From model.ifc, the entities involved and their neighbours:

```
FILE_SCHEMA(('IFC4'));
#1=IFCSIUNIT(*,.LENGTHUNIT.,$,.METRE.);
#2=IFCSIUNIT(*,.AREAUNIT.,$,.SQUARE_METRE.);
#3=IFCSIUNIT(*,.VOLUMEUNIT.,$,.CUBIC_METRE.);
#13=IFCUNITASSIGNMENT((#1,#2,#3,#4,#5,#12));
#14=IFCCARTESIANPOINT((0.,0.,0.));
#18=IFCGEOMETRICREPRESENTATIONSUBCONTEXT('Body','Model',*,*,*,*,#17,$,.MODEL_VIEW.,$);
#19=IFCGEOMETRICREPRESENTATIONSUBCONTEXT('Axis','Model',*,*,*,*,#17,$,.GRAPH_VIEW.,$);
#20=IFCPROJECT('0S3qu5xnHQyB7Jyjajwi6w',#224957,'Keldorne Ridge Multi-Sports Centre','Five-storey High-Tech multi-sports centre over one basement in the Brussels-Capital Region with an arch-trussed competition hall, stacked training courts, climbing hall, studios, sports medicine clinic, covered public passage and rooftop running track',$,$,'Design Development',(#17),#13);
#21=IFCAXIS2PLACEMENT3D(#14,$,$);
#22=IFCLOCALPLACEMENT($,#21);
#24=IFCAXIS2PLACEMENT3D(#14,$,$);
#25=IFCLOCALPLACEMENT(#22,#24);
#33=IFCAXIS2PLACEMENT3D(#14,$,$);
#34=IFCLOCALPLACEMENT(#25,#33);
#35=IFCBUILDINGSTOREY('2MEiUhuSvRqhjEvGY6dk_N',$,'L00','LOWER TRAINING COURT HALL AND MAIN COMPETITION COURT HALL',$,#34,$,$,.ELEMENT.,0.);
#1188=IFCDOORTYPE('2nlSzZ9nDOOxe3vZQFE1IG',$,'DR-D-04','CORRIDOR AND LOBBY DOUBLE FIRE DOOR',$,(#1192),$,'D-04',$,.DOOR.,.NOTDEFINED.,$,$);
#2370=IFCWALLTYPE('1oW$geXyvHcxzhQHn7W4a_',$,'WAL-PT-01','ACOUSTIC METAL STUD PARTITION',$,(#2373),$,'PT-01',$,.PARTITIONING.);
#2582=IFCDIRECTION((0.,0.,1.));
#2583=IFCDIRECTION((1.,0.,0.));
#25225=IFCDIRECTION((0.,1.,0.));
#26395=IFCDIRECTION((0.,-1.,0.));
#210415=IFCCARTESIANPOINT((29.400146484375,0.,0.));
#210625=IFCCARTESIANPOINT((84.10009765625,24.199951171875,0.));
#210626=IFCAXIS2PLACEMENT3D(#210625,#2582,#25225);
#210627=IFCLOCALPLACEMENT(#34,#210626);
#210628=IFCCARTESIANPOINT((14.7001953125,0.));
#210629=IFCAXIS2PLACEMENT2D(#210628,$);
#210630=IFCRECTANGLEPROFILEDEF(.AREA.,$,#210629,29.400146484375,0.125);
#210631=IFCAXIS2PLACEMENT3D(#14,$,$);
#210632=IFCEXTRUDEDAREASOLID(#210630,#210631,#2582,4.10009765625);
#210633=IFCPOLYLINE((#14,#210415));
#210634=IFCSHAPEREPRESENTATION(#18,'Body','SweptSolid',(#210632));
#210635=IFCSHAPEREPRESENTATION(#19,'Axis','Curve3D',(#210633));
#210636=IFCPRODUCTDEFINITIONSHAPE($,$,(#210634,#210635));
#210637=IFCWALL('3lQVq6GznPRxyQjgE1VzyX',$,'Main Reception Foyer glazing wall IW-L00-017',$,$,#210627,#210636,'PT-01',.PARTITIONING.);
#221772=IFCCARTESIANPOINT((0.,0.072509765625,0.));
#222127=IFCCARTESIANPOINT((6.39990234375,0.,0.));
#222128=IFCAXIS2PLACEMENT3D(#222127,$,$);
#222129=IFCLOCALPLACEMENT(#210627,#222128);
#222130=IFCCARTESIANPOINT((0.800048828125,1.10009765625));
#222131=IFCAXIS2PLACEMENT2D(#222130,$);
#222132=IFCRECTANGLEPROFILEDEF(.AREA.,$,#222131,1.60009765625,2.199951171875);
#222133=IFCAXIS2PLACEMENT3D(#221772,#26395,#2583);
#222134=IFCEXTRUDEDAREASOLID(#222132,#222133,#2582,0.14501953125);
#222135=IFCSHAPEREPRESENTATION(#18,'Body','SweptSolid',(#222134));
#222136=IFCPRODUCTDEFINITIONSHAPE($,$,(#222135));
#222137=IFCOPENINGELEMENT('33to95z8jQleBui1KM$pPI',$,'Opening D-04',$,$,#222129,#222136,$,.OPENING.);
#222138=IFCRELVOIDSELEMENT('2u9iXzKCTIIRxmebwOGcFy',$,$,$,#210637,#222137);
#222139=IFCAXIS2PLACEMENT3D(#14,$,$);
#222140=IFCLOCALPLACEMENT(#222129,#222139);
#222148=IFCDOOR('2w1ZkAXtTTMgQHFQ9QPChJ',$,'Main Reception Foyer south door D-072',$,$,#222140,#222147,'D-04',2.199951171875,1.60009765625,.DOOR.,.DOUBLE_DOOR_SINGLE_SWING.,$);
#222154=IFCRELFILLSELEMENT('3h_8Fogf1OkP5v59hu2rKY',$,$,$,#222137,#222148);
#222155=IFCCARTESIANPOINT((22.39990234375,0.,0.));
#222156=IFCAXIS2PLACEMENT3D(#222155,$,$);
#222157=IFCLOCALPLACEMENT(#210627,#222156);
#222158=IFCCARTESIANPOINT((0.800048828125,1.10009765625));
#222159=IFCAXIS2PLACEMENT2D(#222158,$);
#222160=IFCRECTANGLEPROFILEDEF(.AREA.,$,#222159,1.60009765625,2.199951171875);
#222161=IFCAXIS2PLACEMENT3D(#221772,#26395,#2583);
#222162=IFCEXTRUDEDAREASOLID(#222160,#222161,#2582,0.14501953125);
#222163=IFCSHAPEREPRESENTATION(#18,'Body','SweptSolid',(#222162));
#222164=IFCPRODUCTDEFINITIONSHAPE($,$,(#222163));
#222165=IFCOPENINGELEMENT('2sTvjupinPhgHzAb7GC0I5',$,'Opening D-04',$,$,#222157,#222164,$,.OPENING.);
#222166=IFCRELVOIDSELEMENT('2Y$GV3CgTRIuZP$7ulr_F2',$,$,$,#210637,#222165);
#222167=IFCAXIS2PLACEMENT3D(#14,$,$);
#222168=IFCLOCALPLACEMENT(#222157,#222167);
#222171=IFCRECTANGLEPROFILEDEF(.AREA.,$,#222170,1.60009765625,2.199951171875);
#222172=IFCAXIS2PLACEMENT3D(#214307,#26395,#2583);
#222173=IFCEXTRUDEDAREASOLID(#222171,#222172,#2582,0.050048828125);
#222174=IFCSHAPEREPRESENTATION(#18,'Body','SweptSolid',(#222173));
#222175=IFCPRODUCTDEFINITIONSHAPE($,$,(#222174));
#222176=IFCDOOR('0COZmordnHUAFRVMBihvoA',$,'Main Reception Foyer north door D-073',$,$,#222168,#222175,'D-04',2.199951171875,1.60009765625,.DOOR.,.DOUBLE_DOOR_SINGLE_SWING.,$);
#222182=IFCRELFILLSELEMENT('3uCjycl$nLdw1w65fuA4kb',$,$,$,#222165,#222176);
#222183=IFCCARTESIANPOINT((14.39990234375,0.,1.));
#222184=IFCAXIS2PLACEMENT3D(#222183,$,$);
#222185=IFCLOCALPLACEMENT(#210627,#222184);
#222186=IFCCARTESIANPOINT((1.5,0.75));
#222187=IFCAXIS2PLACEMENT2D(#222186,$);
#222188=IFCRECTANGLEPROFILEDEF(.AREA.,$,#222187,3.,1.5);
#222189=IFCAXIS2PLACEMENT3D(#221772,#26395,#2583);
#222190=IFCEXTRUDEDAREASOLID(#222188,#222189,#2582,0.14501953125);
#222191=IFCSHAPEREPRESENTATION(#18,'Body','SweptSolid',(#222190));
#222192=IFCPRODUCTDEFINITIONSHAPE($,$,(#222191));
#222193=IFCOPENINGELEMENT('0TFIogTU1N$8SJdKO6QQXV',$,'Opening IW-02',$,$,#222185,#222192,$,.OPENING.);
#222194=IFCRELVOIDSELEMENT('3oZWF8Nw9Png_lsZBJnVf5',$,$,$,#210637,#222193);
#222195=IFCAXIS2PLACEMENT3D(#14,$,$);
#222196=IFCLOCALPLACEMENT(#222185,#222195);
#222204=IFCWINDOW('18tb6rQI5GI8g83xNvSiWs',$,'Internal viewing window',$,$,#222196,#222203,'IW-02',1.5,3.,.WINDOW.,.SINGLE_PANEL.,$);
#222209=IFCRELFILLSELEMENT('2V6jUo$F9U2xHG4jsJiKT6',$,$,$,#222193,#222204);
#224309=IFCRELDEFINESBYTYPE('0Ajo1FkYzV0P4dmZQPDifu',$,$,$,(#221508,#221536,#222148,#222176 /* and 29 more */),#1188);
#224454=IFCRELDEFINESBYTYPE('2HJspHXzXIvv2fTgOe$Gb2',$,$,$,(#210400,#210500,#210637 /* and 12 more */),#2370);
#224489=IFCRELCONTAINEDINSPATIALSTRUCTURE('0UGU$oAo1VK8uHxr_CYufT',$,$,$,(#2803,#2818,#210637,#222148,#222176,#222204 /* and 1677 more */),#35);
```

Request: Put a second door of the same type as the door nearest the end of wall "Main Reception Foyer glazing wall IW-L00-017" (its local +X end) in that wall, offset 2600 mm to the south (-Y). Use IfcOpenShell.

```python
import ifcopenshell
import ifcopenshell.api.feature
import ifcopenshell.api.geometry
import ifcopenshell.api.root
import ifcopenshell.geom
import ifcopenshell.util.element
import ifcopenshell.util.placement
import ifcopenshell.util.shape
import ifcopenshell.util.unit

model = ifcopenshell.open("model.ifc")
unit_scale = ifcopenshell.util.unit.calculate_unit_scale(model)
settings = ifcopenshell.geom.settings()


def volume(element):
    """Net volume in cubic metres, openings subtracted."""
    shape = ifcopenshell.geom.create_shape(settings, element)
    return ifcopenshell.util.shape.get_volume(shape.geometry)


door = model.by_guid("0COZmordnHUAFRVMBihvoA")
opening = door.FillsVoids[0].RelatingOpeningElement
wall = opening.VoidsElements[0].RelatingBuildingElement
before = volume(wall)
shift = ifcopenshell.util.placement.get_local_placement(wall.ObjectPlacement)[:3, 0] * -2.6 / unit_scale

# copy_class copies the void relationship, type, container and properties, but no geometry.
new_opening = ifcopenshell.api.root.copy_class(model, product=opening)
new_opening.Representation = ifcopenshell.util.element.copy_deep(
    model, opening.Representation, exclude=["IfcGeometricRepresentationContext", "IfcRepresentationMap"]
)
new_door = ifcopenshell.api.root.copy_class(model, product=door)
new_door.Representation = ifcopenshell.util.element.copy_deep(
    model, door.Representation, exclude=["IfcGeometricRepresentationContext", "IfcRepresentationMap"]
)
new_door.Tag = None
ifcopenshell.api.feature.add_filling(model, opening=new_opening, element=new_door)

for old, new in ((opening, new_opening), (door, new_door)):
    matrix = ifcopenshell.util.placement.get_local_placement(old.ObjectPlacement)
    matrix[:3, 3] += shift
    ifcopenshell.api.geometry.edit_object_placement(model, product=new, matrix=matrix, is_si=False)

after = volume(wall)

print(f"wall volume {before:.3f} -> {after:.3f} m3")

model.write("model_edited.ifc")
```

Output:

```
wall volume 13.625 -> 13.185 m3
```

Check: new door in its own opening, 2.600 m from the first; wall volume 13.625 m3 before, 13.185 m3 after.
